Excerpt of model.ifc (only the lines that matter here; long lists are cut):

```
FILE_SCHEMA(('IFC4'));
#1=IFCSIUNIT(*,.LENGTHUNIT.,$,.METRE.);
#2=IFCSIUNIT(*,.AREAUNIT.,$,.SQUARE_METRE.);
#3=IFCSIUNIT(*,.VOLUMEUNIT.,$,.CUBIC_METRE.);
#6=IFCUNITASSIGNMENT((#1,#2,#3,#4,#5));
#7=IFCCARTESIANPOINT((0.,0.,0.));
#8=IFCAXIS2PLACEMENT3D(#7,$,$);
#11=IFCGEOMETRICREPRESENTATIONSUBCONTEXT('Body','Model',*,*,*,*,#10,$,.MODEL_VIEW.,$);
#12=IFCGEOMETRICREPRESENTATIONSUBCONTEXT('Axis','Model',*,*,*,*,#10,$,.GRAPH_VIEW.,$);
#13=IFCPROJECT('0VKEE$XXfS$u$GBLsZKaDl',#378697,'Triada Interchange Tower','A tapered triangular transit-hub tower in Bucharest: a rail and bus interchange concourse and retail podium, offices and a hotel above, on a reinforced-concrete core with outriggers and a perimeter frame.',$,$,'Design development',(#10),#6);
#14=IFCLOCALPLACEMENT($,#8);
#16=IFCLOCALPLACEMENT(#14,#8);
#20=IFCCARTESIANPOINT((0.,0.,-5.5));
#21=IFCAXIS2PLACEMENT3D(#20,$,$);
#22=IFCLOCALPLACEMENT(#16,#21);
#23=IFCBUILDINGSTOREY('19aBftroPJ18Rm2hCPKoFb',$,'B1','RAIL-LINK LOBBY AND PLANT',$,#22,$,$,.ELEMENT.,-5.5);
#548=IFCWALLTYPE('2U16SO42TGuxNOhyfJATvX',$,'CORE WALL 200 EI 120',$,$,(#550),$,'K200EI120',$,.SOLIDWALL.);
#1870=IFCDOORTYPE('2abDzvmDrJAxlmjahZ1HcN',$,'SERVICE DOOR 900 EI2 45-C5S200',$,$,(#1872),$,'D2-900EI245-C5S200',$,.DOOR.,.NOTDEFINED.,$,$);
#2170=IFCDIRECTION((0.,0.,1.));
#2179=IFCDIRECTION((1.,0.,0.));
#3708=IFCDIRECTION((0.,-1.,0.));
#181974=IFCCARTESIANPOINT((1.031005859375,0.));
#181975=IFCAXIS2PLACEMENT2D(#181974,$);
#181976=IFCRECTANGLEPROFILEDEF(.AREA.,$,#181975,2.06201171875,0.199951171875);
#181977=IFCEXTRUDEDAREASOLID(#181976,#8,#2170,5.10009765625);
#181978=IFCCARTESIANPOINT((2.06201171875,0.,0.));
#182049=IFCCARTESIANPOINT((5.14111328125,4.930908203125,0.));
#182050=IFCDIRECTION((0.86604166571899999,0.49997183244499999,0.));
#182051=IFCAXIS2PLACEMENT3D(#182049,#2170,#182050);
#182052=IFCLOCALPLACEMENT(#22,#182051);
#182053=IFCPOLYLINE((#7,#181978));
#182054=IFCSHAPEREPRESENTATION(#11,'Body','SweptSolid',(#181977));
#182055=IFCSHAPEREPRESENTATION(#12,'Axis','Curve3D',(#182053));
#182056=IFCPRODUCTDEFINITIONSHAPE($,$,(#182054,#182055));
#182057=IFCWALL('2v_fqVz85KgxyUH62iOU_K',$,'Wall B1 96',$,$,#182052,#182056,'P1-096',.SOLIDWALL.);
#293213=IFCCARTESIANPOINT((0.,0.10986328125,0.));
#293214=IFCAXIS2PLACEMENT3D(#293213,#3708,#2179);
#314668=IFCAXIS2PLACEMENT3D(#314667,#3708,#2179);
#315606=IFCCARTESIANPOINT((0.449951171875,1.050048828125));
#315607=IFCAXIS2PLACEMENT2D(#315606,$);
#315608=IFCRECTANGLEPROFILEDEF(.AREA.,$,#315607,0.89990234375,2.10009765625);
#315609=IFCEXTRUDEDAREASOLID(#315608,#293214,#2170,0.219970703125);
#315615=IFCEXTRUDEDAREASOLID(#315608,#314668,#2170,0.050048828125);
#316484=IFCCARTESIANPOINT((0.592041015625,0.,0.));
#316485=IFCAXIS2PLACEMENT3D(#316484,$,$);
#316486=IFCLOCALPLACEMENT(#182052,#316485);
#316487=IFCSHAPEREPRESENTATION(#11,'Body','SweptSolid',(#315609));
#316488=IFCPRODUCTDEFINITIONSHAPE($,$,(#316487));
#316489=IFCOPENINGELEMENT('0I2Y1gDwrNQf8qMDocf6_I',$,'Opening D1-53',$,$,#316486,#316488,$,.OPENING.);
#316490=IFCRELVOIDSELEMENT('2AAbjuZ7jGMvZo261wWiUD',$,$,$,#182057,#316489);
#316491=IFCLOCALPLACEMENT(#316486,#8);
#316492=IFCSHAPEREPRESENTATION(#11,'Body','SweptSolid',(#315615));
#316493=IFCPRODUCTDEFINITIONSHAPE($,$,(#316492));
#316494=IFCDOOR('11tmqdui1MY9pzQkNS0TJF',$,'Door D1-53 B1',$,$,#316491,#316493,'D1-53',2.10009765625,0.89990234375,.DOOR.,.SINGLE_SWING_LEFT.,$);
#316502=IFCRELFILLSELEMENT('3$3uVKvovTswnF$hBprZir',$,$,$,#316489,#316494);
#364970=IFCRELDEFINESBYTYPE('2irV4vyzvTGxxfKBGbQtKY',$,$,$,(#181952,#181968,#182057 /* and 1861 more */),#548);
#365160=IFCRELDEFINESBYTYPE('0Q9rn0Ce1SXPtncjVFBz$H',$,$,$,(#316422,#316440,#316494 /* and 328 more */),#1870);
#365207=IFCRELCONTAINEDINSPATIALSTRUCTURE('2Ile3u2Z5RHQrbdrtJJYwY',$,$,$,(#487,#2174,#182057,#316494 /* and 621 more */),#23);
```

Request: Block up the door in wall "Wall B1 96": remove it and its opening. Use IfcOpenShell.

```python
import ifcopenshell
import ifcopenshell.api.feature
import ifcopenshell.api.root
import ifcopenshell.geom
import ifcopenshell.util.shape

model = ifcopenshell.open("model.ifc")
settings = ifcopenshell.geom.settings()


def volume(element):
    """Net volume in cubic metres, openings subtracted."""
    shape = ifcopenshell.geom.create_shape(settings, element)
    return ifcopenshell.util.shape.get_volume(shape.geometry)


door = model.by_guid("11tmqdui1MY9pzQkNS0TJF")
opening = door.FillsVoids[0].RelatingOpeningElement
wall = opening.VoidsElements[0].RelatingBuildingElement
before = volume(wall)

ifcopenshell.api.root.remove_product(model, product=door)
ifcopenshell.api.feature.remove_feature(model, feature=opening)

after = volume(wall)

print(f"wall volume {before:.3f} -> {after:.3f} m3")

model.write("model_updated.ifc")
```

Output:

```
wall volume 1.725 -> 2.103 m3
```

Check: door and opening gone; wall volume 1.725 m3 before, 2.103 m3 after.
